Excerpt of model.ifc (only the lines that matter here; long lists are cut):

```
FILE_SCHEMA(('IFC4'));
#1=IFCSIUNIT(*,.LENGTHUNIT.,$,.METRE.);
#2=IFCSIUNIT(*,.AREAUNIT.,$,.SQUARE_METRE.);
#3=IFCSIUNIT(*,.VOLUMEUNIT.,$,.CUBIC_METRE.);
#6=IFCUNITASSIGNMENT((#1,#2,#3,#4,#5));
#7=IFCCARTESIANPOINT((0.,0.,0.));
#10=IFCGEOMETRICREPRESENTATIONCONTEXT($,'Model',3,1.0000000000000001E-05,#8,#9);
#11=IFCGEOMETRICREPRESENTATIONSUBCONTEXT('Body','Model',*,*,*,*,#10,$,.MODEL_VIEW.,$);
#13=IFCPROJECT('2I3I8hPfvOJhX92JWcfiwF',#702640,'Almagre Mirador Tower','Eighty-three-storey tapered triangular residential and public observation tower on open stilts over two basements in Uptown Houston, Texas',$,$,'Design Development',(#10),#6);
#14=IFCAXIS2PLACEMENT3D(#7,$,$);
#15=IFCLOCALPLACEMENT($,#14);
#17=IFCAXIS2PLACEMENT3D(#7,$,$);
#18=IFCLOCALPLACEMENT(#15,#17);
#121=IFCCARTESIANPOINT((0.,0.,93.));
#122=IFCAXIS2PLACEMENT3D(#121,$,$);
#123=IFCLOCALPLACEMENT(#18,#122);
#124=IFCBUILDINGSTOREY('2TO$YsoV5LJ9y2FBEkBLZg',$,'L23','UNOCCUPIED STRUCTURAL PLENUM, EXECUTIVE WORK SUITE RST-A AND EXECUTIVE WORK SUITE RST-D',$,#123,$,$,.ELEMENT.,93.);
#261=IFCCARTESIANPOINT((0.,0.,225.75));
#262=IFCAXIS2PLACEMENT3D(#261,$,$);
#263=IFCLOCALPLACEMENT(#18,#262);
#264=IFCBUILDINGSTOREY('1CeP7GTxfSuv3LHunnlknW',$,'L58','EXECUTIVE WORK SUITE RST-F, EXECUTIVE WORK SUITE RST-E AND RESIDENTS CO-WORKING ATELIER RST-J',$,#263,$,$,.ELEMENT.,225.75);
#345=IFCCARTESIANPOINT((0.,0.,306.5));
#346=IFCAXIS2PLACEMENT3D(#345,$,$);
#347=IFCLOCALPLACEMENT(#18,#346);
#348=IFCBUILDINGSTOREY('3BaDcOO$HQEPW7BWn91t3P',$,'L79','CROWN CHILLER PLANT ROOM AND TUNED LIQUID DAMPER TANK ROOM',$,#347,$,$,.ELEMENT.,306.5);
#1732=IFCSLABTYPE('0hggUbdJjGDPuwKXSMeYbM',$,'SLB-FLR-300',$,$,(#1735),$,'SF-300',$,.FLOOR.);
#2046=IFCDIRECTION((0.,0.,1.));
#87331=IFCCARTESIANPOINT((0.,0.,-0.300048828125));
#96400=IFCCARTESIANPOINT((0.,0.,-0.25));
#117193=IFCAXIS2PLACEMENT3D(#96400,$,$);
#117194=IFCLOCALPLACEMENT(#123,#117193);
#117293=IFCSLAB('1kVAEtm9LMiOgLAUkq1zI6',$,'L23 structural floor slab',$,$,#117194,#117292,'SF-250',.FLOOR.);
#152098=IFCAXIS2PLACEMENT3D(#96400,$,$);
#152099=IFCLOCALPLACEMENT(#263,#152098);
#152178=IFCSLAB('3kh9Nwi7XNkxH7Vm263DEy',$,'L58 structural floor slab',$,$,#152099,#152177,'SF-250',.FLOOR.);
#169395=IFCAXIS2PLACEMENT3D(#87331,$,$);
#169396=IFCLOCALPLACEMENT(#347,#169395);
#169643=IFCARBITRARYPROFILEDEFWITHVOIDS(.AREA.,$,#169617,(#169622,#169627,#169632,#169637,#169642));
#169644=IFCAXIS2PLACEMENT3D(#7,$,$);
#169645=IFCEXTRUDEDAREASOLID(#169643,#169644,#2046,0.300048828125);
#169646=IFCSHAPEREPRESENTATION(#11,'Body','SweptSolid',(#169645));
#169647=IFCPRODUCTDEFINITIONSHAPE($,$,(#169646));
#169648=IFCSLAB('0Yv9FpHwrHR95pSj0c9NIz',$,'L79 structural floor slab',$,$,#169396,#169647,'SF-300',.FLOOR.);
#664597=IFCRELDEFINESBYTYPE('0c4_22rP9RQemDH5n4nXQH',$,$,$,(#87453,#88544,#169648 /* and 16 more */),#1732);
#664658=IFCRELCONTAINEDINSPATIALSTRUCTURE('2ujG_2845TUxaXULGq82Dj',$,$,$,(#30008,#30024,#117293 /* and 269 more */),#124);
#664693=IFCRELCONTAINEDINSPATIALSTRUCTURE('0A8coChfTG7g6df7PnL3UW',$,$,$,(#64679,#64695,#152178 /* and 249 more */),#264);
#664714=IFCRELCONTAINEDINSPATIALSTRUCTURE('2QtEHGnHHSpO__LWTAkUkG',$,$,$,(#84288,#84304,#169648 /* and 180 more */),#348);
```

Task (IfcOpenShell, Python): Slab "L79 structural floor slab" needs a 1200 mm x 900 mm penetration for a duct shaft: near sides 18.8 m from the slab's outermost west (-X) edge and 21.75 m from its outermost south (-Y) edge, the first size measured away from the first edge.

```python
import numpy as np
import ifcopenshell
import ifcopenshell.api.feature
import ifcopenshell.api.geometry
import ifcopenshell.api.root
import ifcopenshell.geom
import ifcopenshell.util.placement
import ifcopenshell.util.representation
import ifcopenshell.util.shape
import ifcopenshell.util.unit

model = ifcopenshell.open("model.ifc")
unit_scale = ifcopenshell.util.unit.calculate_unit_scale(model)
settings = ifcopenshell.geom.settings()


def volume(element):
    """Net volume in cubic metres, openings subtracted."""
    shape = ifcopenshell.geom.create_shape(settings, element)
    return ifcopenshell.util.shape.get_volume(shape.geometry)


slab = model.by_guid("0Yv9FpHwrHR95pSj0c9NIz")
before = volume(slab)

# Extent in the slab's own axes, in metres. The edges named are its -X and -Y sides.
slab_shape = ifcopenshell.geom.create_shape(settings, slab)
vertices = ifcopenshell.util.shape.get_vertices(slab_shape.geometry)
x_min, y_min, bottom = vertices.min(axis=0)
top = vertices[:, 2].max()

opening = ifcopenshell.api.root.create_entity(model, ifc_class="IfcOpeningElement", name="Duct shaft opening", predefined_type="OPENING")
context = ifcopenshell.util.representation.get_context(model, "Model", "Body", "MODEL_VIEW")
width, depth = 1.2, 0.9
outline = [(0.0, 0.0), (width, 0.0), (width, depth), (0.0, depth), (0.0, 0.0)]
# Overshoot both faces by 50 mm so the cut is clean.
shape = ifcopenshell.api.geometry.add_slab_representation(
    model, context=context, depth=top - bottom + 0.1, polyline=outline
)
ifcopenshell.api.geometry.assign_representation(model, product=opening, representation=shape)

matrix = ifcopenshell.util.placement.get_local_placement(slab.ObjectPlacement)
matrix[:, 3] = matrix @ np.append(np.array([x_min + 18.8, y_min + 21.75, bottom - 0.05]) / unit_scale, 1.0)
ifcopenshell.api.geometry.edit_object_placement(model, product=opening, matrix=matrix, is_si=False)
ifcopenshell.api.feature.add_feature(model, feature=opening, element=slab)

after = volume(slab)

print(f"slab volume {before:.3f} -> {after:.3f} m3")

model.write("model-out.ifc")
```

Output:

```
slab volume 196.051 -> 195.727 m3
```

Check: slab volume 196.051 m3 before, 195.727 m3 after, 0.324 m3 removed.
